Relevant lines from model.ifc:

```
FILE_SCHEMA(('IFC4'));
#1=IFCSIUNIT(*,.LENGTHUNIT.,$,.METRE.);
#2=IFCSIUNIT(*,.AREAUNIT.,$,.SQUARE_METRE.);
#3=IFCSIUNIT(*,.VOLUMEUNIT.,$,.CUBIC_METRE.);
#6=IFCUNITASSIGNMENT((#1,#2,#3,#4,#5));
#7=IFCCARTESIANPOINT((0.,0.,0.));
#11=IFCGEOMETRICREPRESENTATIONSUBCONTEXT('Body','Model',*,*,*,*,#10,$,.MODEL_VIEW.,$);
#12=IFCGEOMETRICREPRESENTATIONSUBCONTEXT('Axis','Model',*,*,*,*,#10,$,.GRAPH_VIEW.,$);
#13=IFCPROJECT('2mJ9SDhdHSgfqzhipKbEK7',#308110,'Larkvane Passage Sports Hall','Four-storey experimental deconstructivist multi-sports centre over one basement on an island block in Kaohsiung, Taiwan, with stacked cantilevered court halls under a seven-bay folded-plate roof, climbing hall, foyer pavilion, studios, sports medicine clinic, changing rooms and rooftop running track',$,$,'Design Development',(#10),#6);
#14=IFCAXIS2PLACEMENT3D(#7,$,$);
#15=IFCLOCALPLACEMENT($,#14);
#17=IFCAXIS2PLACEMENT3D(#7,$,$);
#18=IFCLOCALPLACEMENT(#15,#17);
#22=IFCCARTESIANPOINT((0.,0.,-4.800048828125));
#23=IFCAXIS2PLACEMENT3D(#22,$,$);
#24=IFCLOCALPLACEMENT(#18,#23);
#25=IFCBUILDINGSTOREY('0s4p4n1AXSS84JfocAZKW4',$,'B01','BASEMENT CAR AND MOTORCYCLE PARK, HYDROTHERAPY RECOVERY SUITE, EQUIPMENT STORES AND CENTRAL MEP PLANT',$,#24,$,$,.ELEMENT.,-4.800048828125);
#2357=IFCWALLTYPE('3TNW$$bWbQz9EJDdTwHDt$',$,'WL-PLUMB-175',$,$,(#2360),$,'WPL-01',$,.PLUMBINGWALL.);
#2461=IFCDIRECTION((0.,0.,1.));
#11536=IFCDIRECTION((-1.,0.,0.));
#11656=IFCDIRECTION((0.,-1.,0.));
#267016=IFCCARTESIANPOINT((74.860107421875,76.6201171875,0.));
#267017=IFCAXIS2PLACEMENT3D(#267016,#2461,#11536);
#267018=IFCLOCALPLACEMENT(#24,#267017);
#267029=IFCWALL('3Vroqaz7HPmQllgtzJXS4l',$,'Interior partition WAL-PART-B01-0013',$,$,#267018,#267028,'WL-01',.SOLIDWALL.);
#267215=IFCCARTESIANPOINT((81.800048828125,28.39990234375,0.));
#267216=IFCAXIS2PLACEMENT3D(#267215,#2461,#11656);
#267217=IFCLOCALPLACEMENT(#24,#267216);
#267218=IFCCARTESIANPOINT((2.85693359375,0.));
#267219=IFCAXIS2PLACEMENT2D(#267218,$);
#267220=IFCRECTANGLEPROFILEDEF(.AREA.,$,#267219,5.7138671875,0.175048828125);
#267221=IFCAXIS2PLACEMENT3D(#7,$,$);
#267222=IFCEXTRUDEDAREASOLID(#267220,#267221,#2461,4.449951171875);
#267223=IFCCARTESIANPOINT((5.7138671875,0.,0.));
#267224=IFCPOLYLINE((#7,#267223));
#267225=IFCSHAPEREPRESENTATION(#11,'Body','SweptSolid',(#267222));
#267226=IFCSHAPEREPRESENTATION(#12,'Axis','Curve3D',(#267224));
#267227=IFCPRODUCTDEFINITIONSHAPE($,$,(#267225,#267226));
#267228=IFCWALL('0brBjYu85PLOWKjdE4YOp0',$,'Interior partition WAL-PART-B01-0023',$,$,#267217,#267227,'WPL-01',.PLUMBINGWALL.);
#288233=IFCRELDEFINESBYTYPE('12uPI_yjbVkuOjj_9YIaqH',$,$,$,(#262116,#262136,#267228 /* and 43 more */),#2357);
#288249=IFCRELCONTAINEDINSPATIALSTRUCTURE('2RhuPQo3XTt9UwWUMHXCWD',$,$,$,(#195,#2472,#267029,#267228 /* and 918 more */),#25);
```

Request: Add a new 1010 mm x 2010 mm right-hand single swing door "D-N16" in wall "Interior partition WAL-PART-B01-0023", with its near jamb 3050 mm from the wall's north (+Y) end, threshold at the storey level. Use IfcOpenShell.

```python
import numpy as np
import ifcopenshell
import ifcopenshell.api.feature
import ifcopenshell.api.geometry
import ifcopenshell.api.root
import ifcopenshell.api.spatial
import ifcopenshell.geom
import ifcopenshell.util.element
import ifcopenshell.util.placement
import ifcopenshell.util.representation
import ifcopenshell.util.shape
import ifcopenshell.util.unit

model = ifcopenshell.open("model.ifc")
unit_scale = ifcopenshell.util.unit.calculate_unit_scale(model)
settings = ifcopenshell.geom.settings()


def volume(element):
    """Net volume in cubic metres, openings subtracted."""
    shape = ifcopenshell.geom.create_shape(settings, element)
    return ifcopenshell.util.shape.get_volume(shape.geometry)


wall = model.by_id(267228)
storey = ifcopenshell.util.element.get_container(wall, ifc_class="IfcBuildingStorey")
context = ifcopenshell.util.representation.get_context(model, "Model", "Body", "MODEL_VIEW")
before = volume(wall)

width, height, from_end, sill = 1.01, 2.01, 3.05, 0.0  # metres

# The wall runs along its own X axis, and the end named is its -X end.
wall_shape = ifcopenshell.geom.create_shape(settings, wall)
x, y, z = ifcopenshell.util.shape.get_vertices(wall_shape.geometry).T
start = x.min() + from_end
face, thickness = float(y.min()), float(y.max() - y.min())
wall_matrix = ifcopenshell.util.placement.get_local_placement(wall.ObjectPlacement)
level = ifcopenshell.util.placement.get_local_placement(storey.ObjectPlacement)[2, 3]


def in_wall(x, y):
    """Placement at x, y metres in the wall's axes, at sill height."""
    matrix = wall_matrix.copy()
    matrix[:, 3] = wall_matrix @ np.array([x / unit_scale, y / unit_scale, 0.0, 1.0])
    matrix[2, 3] = level + sill / unit_scale
    return matrix


# Opening: a box that overshoots both wall faces by 50 mm.
opening = ifcopenshell.api.root.create_entity(model, ifc_class="IfcOpeningElement", predefined_type="OPENING")
box = ifcopenshell.api.geometry.add_wall_representation(
    model, context=context, length=width, height=height, thickness=thickness + 0.1
)
ifcopenshell.api.geometry.assign_representation(model, product=opening, representation=box)
ifcopenshell.api.geometry.edit_object_placement(model, product=opening, matrix=in_wall(start, face - 0.05), is_si=False)
ifcopenshell.api.feature.add_feature(model, feature=opening, element=wall)

door = ifcopenshell.api.root.create_entity(model, ifc_class="IfcDoor", name="D-N16", predefined_type="DOOR")
door.OverallWidth, door.OverallHeight = width / unit_scale, height / unit_scale
door.OperationType = "SINGLE_SWING_RIGHT"
body = ifcopenshell.api.geometry.add_door_representation(
    model,
    context=context,
    overall_width=door.OverallWidth,
    overall_height=door.OverallHeight,
    operation_type="SINGLE_SWING_RIGHT",
    lining_properties={"LiningDepth": thickness / unit_scale, "ThresholdDepth": thickness / unit_scale},
)
ifcopenshell.api.geometry.assign_representation(model, product=door, representation=body)
ifcopenshell.api.spatial.assign_container(model, products=[door], relating_structure=storey)
ifcopenshell.api.feature.add_filling(model, opening=opening, element=door)

# The lining spans the wall, so the door starts at the wall face.
ifcopenshell.api.geometry.edit_object_placement(model, product=door, matrix=in_wall(start, face), is_si=False)

after = volume(wall)

print(f"wall volume {before:.3f} -> {after:.3f} m3")

model.write("model_rev.ifc")
```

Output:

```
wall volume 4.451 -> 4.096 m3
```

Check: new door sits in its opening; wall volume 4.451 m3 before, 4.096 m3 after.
